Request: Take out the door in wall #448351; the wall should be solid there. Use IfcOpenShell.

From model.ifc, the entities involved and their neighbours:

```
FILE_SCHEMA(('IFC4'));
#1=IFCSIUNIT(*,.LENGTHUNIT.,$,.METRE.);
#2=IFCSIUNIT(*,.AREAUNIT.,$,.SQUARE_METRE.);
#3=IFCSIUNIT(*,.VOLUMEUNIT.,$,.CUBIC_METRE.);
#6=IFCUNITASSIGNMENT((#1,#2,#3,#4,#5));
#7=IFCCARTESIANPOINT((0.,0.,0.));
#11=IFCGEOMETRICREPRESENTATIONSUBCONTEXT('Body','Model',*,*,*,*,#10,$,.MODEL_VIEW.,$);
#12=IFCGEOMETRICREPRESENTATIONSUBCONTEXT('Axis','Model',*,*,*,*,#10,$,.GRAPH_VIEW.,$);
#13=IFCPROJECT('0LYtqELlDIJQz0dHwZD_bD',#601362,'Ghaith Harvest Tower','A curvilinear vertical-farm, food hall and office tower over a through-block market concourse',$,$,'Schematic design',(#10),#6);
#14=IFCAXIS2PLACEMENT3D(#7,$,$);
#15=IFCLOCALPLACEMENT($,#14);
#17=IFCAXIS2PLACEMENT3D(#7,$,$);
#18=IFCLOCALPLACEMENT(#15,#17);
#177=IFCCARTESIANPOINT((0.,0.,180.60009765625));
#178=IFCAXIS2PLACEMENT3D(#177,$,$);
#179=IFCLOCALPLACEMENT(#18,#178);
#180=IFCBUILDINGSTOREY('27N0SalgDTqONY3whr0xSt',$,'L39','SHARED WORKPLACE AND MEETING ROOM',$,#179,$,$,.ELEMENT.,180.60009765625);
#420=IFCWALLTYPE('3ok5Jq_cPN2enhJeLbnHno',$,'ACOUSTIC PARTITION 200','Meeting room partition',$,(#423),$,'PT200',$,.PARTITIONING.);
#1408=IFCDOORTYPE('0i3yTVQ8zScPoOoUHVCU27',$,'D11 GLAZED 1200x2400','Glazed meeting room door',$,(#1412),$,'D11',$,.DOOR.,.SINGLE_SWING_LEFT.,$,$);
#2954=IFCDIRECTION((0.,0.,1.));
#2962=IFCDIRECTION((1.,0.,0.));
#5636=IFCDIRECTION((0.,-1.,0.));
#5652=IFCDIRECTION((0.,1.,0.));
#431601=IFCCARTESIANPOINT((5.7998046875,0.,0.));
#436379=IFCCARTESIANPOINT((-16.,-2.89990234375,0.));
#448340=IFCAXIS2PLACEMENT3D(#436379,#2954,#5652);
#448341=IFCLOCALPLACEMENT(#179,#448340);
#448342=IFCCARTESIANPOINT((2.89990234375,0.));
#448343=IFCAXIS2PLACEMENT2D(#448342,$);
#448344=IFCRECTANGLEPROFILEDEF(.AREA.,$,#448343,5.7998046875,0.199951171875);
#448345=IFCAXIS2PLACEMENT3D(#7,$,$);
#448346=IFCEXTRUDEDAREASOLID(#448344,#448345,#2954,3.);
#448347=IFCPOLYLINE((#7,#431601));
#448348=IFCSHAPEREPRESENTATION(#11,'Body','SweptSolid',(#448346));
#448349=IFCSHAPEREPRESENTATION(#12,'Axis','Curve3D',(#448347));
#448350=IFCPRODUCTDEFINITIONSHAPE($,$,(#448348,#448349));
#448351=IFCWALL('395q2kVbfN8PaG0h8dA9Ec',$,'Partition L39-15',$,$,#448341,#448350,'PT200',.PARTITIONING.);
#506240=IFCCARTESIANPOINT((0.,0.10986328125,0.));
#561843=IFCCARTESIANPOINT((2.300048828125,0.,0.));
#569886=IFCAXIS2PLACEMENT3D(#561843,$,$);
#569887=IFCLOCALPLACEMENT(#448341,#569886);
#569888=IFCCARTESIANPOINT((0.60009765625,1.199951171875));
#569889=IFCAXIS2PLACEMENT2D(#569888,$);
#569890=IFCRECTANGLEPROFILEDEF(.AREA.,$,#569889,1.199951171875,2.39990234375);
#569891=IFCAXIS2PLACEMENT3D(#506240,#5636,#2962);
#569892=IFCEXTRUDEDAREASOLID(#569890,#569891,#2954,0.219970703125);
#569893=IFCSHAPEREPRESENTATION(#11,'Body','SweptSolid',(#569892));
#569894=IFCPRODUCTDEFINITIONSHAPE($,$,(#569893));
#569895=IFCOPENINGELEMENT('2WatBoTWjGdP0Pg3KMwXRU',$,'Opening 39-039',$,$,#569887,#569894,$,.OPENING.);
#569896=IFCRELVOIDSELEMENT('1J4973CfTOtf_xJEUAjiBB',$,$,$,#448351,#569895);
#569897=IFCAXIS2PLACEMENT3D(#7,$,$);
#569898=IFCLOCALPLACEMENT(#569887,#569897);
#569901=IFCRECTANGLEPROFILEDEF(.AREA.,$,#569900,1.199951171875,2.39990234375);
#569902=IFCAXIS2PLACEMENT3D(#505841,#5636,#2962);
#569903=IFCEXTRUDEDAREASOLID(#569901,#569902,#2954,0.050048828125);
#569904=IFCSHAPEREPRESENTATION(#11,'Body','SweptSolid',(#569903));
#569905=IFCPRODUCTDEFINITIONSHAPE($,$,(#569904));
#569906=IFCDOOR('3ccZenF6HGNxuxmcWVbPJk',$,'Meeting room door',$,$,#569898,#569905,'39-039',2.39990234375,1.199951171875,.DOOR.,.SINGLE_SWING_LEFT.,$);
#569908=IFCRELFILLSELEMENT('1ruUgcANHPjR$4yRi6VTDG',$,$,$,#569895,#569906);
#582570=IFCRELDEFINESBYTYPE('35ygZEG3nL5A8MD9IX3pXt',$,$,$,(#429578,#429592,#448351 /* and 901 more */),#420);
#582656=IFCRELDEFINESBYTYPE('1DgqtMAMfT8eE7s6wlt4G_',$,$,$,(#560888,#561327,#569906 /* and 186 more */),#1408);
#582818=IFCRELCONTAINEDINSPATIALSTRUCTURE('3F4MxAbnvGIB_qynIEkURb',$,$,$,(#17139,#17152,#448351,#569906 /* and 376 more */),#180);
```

```python
import ifcopenshell
import ifcopenshell.api.feature
import ifcopenshell.api.root
import ifcopenshell.geom
import ifcopenshell.util.shape

model = ifcopenshell.open("model.ifc")
settings = ifcopenshell.geom.settings()


def volume(element):
    """Net volume in cubic metres, openings subtracted."""
    shape = ifcopenshell.geom.create_shape(settings, element)
    return ifcopenshell.util.shape.get_volume(shape.geometry)


door = model.by_guid("3ccZenF6HGNxuxmcWVbPJk")
opening = door.FillsVoids[0].RelatingOpeningElement
wall = opening.VoidsElements[0].RelatingBuildingElement
before = volume(wall)

ifcopenshell.api.root.remove_product(model, product=door)
ifcopenshell.api.feature.remove_feature(model, feature=opening)

after = volume(wall)

print(f"wall volume {before:.3f} -> {after:.3f} m3")

model.write("model_v2.ifc")
```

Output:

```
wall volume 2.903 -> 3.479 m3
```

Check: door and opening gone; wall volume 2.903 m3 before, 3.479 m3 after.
